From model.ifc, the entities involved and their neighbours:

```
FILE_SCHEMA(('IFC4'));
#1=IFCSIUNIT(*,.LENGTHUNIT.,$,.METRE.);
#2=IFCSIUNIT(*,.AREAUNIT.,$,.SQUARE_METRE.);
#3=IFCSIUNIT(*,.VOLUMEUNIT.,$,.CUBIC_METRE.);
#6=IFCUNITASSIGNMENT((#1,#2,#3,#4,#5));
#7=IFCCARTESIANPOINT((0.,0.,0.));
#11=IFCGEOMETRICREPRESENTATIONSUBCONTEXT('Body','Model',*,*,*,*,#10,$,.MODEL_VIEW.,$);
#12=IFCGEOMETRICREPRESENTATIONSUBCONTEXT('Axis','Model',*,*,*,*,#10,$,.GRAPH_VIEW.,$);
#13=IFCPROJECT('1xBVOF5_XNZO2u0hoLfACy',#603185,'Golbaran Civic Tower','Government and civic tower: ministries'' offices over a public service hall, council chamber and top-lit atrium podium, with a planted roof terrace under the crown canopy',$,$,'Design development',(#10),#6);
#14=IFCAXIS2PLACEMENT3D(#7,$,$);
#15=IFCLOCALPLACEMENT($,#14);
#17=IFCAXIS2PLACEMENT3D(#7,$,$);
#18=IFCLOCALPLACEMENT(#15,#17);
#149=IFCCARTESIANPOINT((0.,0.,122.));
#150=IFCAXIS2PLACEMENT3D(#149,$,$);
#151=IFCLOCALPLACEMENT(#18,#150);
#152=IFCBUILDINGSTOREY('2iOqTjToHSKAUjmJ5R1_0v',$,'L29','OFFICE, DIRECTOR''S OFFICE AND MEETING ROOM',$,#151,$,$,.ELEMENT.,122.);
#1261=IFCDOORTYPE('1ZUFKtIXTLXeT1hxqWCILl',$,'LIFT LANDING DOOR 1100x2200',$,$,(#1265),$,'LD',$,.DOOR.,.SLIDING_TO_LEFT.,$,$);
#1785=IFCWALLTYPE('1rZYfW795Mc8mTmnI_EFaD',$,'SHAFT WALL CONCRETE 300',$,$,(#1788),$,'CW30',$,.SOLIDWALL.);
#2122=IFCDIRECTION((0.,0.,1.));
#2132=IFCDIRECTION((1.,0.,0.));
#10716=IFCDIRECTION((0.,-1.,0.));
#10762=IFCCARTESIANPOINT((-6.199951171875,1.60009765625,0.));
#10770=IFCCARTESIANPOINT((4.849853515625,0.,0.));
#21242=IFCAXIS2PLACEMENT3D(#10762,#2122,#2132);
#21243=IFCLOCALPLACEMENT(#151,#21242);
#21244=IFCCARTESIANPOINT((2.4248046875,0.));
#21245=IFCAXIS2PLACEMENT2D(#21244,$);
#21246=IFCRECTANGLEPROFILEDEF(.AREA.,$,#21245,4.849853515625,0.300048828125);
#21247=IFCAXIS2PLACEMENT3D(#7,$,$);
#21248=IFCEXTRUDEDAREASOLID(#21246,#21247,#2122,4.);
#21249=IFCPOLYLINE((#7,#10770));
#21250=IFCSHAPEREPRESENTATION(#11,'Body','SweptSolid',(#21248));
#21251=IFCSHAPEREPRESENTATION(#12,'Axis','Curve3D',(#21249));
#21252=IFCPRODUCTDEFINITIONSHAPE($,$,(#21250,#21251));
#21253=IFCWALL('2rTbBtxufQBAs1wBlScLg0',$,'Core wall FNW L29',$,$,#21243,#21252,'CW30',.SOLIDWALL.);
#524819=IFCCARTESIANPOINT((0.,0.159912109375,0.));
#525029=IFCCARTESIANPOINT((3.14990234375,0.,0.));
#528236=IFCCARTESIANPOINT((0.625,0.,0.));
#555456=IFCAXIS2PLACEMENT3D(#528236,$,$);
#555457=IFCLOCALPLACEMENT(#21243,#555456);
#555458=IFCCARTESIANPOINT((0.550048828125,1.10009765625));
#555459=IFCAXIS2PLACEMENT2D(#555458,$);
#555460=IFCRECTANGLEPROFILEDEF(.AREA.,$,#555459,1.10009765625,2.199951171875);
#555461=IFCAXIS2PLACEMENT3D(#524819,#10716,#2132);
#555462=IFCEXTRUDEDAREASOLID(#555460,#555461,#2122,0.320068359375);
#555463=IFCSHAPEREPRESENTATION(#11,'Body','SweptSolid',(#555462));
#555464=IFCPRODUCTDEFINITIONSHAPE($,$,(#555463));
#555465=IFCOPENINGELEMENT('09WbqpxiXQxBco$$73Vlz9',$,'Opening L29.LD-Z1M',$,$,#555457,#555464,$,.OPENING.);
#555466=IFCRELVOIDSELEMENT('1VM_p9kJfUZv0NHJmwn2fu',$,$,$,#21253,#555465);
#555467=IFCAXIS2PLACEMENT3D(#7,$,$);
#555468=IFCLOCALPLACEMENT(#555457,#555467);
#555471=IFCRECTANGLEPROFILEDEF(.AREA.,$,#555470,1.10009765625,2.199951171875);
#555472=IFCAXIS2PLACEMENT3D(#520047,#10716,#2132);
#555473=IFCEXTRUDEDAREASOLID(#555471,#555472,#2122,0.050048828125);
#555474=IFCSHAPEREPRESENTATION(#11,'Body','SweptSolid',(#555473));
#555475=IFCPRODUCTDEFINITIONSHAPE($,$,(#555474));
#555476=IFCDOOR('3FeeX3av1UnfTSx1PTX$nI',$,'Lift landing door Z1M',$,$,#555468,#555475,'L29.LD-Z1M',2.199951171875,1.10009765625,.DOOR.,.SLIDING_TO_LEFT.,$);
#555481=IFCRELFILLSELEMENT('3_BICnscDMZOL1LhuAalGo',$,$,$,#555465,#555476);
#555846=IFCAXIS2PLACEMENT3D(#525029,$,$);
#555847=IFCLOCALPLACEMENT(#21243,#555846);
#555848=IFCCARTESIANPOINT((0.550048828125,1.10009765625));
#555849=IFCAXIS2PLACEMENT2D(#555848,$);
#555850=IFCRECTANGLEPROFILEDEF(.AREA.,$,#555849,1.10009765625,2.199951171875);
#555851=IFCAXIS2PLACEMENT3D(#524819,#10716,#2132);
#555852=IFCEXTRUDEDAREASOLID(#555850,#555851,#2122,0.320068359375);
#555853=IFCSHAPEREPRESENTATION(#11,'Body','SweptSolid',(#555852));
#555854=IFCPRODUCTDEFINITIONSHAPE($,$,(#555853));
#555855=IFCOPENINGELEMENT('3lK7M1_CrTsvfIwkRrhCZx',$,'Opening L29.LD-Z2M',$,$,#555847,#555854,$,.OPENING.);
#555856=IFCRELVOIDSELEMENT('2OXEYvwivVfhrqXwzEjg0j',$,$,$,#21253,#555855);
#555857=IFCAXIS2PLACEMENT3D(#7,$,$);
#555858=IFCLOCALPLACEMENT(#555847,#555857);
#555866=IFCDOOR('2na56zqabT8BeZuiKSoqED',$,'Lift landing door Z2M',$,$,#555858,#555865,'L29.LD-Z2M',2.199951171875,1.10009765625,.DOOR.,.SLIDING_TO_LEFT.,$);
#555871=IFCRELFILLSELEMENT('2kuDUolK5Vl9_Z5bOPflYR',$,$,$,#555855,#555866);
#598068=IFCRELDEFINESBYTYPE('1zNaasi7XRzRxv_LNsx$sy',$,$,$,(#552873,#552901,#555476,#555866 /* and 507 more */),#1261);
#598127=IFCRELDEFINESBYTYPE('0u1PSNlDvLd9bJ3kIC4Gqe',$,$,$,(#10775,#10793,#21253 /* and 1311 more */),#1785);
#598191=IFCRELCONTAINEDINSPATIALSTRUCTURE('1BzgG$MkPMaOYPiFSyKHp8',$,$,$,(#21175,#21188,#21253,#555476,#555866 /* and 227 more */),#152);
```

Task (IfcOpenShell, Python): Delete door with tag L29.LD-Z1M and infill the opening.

```python
import ifcopenshell
import ifcopenshell.api.feature
import ifcopenshell.api.root
import ifcopenshell.geom
import ifcopenshell.util.shape

model = ifcopenshell.open("model.ifc")
settings = ifcopenshell.geom.settings()


def volume(element):
    """Net volume in cubic metres, openings subtracted."""
    shape = ifcopenshell.geom.create_shape(settings, element)
    return ifcopenshell.util.shape.get_volume(shape.geometry)


door = model.by_guid("3FeeX3av1UnfTSx1PTX$nI")
opening = door.FillsVoids[0].RelatingOpeningElement
wall = opening.VoidsElements[0].RelatingBuildingElement
before = volume(wall)

ifcopenshell.api.root.remove_product(model, product=door)
ifcopenshell.api.feature.remove_feature(model, feature=opening)

after = volume(wall)

print(f"wall volume {before:.3f} -> {after:.3f} m3")

model.write("model_edited.ifc")
```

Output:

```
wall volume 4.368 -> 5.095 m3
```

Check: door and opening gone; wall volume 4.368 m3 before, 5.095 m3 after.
